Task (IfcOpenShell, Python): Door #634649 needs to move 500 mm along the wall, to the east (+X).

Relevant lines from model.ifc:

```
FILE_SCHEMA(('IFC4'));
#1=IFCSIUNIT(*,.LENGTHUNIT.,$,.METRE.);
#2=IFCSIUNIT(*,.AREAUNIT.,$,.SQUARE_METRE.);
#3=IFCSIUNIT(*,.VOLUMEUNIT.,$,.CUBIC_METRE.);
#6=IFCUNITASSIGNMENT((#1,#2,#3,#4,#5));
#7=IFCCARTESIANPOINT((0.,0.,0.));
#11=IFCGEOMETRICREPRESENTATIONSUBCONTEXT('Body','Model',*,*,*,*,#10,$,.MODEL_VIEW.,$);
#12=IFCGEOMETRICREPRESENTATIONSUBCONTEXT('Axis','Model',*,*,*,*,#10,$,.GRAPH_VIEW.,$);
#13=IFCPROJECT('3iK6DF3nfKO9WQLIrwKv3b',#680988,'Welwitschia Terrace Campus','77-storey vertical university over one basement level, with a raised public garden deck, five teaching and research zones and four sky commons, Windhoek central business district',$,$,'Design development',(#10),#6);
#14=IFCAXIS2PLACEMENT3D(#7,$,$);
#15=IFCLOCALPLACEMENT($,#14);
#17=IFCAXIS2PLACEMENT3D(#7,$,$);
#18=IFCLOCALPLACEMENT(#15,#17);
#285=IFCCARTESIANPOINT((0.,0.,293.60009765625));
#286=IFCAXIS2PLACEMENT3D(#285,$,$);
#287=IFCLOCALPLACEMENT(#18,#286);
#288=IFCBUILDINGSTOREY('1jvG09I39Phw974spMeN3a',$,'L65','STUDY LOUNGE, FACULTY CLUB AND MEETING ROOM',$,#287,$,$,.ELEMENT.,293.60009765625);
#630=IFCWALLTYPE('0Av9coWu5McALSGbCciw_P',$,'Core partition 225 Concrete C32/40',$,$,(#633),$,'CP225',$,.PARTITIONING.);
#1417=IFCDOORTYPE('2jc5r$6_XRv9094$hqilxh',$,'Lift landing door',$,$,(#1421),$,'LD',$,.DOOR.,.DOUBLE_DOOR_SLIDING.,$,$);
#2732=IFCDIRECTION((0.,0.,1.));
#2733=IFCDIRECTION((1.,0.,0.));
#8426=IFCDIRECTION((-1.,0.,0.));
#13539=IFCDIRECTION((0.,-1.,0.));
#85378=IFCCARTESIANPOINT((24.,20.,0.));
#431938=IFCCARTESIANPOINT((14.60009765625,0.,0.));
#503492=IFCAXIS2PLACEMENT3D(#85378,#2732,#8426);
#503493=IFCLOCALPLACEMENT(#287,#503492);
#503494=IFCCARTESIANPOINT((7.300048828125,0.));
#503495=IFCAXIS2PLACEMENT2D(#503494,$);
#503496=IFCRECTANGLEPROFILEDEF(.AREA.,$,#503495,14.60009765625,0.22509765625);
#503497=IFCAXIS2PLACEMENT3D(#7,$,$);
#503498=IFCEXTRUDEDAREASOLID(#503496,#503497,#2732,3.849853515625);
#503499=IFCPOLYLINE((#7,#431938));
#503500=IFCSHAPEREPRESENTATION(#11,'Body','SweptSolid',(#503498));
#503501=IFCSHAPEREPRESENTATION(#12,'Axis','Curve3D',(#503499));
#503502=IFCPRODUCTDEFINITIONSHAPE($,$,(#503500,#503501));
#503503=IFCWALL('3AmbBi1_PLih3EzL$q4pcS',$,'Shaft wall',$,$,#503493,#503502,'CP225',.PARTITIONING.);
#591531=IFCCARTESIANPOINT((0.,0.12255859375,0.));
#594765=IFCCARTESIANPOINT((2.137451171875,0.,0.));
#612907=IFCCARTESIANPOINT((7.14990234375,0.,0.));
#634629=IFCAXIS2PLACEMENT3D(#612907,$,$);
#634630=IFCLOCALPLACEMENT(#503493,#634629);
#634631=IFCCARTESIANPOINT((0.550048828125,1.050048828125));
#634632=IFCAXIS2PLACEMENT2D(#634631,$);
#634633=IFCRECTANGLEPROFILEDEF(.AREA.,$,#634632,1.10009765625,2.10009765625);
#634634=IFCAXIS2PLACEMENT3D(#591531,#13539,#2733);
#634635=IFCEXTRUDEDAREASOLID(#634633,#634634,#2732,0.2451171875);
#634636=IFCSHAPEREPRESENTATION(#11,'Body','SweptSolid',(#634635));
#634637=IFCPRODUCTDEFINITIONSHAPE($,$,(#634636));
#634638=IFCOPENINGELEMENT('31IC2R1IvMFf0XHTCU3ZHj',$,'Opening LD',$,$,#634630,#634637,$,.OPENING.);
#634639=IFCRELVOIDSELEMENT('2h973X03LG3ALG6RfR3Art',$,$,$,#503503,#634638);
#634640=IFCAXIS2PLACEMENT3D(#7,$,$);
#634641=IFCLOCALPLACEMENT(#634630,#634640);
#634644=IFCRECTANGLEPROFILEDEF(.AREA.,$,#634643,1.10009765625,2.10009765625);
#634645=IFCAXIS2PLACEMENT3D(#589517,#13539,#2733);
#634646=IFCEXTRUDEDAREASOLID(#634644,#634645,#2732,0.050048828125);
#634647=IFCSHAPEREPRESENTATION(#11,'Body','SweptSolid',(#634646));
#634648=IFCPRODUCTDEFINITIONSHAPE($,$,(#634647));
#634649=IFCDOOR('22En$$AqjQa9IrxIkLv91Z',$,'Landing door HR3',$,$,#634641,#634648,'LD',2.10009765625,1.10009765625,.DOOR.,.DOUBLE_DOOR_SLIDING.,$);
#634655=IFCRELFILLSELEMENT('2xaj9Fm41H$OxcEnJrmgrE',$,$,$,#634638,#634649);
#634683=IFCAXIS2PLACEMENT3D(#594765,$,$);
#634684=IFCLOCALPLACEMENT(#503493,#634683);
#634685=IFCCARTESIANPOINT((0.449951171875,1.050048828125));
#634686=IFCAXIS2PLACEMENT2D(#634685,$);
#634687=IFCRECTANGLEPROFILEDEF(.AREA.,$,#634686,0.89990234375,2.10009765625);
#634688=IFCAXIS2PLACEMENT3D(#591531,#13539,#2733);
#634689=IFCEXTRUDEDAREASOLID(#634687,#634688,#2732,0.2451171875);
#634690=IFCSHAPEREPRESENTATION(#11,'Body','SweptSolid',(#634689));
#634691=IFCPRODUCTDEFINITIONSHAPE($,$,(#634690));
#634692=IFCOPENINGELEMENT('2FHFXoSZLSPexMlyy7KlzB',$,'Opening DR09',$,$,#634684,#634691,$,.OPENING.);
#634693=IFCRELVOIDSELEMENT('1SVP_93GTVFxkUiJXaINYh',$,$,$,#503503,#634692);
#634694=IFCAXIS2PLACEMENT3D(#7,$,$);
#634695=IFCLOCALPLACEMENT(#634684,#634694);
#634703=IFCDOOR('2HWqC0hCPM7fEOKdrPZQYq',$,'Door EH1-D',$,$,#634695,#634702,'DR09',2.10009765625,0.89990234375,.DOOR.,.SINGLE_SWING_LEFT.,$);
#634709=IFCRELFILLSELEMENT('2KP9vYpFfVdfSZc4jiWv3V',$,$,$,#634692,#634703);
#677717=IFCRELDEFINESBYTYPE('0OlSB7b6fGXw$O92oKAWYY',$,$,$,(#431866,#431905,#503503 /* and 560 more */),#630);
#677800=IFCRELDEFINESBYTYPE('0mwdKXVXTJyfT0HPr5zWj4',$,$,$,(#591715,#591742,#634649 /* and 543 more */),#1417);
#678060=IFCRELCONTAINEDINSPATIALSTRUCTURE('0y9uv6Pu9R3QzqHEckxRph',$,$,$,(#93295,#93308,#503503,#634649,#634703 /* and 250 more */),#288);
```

```python
import ifcopenshell
import ifcopenshell.api.geometry
import ifcopenshell.util.placement
import ifcopenshell.util.unit

model = ifcopenshell.open("model.ifc")
unit_scale = ifcopenshell.util.unit.calculate_unit_scale(model)

door = model.by_guid("22En$$AqjQa9IrxIkLv91Z")
opening = door.FillsVoids[0].RelatingOpeningElement
wall = opening.VoidsElements[0].RelatingBuildingElement

wall_matrix = ifcopenshell.util.placement.get_local_placement(wall.ObjectPlacement)
shift = wall_matrix[:3, 0] * -0.5 / unit_scale
before = ifcopenshell.util.placement.get_local_placement(door.ObjectPlacement)[:3, 3].copy()

# The door is placed relative to its opening, so it follows when the opening moves.
matrix = ifcopenshell.util.placement.get_local_placement(opening.ObjectPlacement)
matrix[:3, 3] += shift
ifcopenshell.api.geometry.edit_object_placement(
    model, product=opening, matrix=matrix, is_si=False, should_transform_children=True
)

after = ifcopenshell.util.placement.get_local_placement(door.ObjectPlacement)[:3, 3]
print("door moved by", (after - before).round(3) + 0.0)

model.write("model_rev.ifc")
```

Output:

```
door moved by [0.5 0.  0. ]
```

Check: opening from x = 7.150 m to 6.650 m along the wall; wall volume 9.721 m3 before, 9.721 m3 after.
